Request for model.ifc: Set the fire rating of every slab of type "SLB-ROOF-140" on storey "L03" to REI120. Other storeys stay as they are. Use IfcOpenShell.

First a look at what the model holds.

```python
import ifcopenshell
import ifcopenshell.util.element

model = ifcopenshell.open("model.ifc")
print(model.schema)
storey = next(s for s in model.by_type("IfcBuildingStorey") if s.Name == "L03")
slabs = [e for e in ifcopenshell.util.element.get_decomposition(storey) if e.is_a("IfcSlab")]
seen = {}
for e in slabs:
    element_type = ifcopenshell.util.element.get_type(e)
    key = (element_type.Name if element_type != e and element_type else None, ifcopenshell.util.element.get_pset(e, "Pset_SlabCommon", "FireRating"))
    seen[key] = seen.get(key, 0) + 1
for (name, value), count in sorted(seen.items(), key=str):
    print(count, "x", name, "|", value)
```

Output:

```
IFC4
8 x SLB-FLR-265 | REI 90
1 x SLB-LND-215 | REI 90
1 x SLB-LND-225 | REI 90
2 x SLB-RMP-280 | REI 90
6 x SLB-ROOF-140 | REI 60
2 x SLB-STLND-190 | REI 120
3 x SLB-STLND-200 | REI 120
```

```python
import ifcopenshell
import ifcopenshell.api.pset
import ifcopenshell.util.element

model = ifcopenshell.open("model.ifc")

storey = next(s for s in model.by_type("IfcBuildingStorey") if s.Name == "L03")
slabs = [e for e in ifcopenshell.util.element.get_decomposition(storey) if e.is_a("IfcSlab")]

count = 0
for e in slabs:
    element_type = ifcopenshell.util.element.get_type(e)
    if element_type in (None, e) or element_type.Name != "SLB-ROOF-140":
        continue
    # add_pset returns the element's existing set when there is one.
    pset = ifcopenshell.api.pset.add_pset(model, product=e, name="Pset_SlabCommon")
    ifcopenshell.api.pset.edit_pset(model, pset=pset, properties={"FireRating": "REI120"})
    count += 1

print(count, "slabs updated")

model.write("model_edited.ifc")
```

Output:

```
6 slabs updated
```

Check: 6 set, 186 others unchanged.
